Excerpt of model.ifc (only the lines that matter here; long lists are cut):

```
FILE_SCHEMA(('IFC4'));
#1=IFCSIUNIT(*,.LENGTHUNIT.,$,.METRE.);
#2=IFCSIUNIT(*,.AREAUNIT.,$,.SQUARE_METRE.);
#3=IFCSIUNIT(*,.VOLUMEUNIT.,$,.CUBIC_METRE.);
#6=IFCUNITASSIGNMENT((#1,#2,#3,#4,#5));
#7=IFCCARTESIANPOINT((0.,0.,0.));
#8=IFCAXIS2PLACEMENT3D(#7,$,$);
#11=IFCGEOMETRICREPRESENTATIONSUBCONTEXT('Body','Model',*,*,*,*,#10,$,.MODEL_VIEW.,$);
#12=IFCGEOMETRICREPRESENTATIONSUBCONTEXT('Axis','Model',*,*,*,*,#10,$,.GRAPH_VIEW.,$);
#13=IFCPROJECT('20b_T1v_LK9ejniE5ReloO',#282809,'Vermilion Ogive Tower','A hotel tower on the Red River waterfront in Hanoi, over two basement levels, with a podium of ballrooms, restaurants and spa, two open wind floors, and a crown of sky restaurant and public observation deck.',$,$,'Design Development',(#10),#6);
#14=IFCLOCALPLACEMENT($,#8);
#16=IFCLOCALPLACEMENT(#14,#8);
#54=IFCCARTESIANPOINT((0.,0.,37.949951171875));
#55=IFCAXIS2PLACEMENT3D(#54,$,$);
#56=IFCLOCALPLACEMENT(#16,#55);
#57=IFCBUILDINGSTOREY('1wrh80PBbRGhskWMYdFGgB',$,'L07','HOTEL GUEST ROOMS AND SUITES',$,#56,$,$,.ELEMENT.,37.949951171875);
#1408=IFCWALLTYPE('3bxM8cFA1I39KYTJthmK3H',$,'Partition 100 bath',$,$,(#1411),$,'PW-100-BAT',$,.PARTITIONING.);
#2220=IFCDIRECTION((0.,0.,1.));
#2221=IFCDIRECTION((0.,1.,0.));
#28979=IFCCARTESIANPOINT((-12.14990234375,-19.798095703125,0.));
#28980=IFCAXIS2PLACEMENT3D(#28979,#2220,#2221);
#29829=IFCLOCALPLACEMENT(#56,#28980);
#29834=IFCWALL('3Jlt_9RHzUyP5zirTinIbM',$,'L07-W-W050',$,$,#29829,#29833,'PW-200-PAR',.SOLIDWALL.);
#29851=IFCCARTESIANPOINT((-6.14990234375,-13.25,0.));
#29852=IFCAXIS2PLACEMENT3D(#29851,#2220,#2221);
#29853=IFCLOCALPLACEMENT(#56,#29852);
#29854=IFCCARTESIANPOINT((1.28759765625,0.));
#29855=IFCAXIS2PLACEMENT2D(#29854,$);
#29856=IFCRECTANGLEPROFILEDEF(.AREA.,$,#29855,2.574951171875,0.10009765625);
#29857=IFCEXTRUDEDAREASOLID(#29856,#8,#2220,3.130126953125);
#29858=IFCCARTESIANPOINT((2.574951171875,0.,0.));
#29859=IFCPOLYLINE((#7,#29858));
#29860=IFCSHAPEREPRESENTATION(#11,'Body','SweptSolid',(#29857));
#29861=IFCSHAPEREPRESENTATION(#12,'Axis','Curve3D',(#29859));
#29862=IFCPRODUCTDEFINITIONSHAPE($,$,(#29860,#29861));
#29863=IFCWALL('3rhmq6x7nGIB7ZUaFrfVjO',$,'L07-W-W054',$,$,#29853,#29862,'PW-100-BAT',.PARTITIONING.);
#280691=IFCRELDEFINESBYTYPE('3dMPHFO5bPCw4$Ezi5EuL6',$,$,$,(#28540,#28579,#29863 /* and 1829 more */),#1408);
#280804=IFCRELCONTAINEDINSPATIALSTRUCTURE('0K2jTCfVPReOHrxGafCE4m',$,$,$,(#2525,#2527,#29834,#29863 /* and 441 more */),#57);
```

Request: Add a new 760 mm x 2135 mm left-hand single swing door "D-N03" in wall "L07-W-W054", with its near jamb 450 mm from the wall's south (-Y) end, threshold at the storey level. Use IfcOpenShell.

```python
import numpy as np
import ifcopenshell
import ifcopenshell.api.feature
import ifcopenshell.api.geometry
import ifcopenshell.api.root
import ifcopenshell.api.spatial
import ifcopenshell.geom
import ifcopenshell.util.element
import ifcopenshell.util.placement
import ifcopenshell.util.representation
import ifcopenshell.util.shape
import ifcopenshell.util.unit

model = ifcopenshell.open("model.ifc")
unit_scale = ifcopenshell.util.unit.calculate_unit_scale(model)
settings = ifcopenshell.geom.settings()


def volume(element):
    """Net volume in cubic metres, openings subtracted."""
    shape = ifcopenshell.geom.create_shape(settings, element)
    return ifcopenshell.util.shape.get_volume(shape.geometry)


wall = model.by_id(29863)
storey = ifcopenshell.util.element.get_container(wall, ifc_class="IfcBuildingStorey")
context = ifcopenshell.util.representation.get_context(model, "Model", "Body", "MODEL_VIEW")
before = volume(wall)

width, height, from_end, sill = 0.76, 2.135, 0.45, 0.0  # metres

# The wall runs along its own X axis, and the end named is its -X end.
wall_shape = ifcopenshell.geom.create_shape(settings, wall)
x, y, z = ifcopenshell.util.shape.get_vertices(wall_shape.geometry).T
start = x.min() + from_end
face, thickness = float(y.min()), float(y.max() - y.min())
wall_matrix = ifcopenshell.util.placement.get_local_placement(wall.ObjectPlacement)
level = ifcopenshell.util.placement.get_local_placement(storey.ObjectPlacement)[2, 3]


def in_wall(x, y):
    """Placement at x, y metres in the wall's axes, at sill height."""
    matrix = wall_matrix.copy()
    matrix[:, 3] = wall_matrix @ np.array([x / unit_scale, y / unit_scale, 0.0, 1.0])
    matrix[2, 3] = level + sill / unit_scale
    return matrix


# Opening: a box that overshoots both wall faces by 50 mm.
opening = ifcopenshell.api.root.create_entity(model, ifc_class="IfcOpeningElement", predefined_type="OPENING")
box = ifcopenshell.api.geometry.add_wall_representation(
    model, context=context, length=width, height=height, thickness=thickness + 0.1
)
ifcopenshell.api.geometry.assign_representation(model, product=opening, representation=box)
ifcopenshell.api.geometry.edit_object_placement(model, product=opening, matrix=in_wall(start, face - 0.05), is_si=False)
ifcopenshell.api.feature.add_feature(model, feature=opening, element=wall)

door = ifcopenshell.api.root.create_entity(model, ifc_class="IfcDoor", name="D-N03", predefined_type="DOOR")
door.OverallWidth, door.OverallHeight = width / unit_scale, height / unit_scale
door.OperationType = "SINGLE_SWING_LEFT"
body = ifcopenshell.api.geometry.add_door_representation(
    model,
    context=context,
    overall_width=door.OverallWidth,
    overall_height=door.OverallHeight,
    operation_type="SINGLE_SWING_LEFT",
    lining_properties={"LiningDepth": thickness / unit_scale, "ThresholdDepth": thickness / unit_scale},
)
ifcopenshell.api.geometry.assign_representation(model, product=door, representation=body)
ifcopenshell.api.spatial.assign_container(model, products=[door], relating_structure=storey)
ifcopenshell.api.feature.add_filling(model, opening=opening, element=door)

# The lining spans the wall, so the door starts at the wall face.
ifcopenshell.api.geometry.edit_object_placement(model, product=door, matrix=in_wall(start, face), is_si=False)

after = volume(wall)

print(f"wall volume {before:.3f} -> {after:.3f} m3")

model.write("model_edited.ifc")
```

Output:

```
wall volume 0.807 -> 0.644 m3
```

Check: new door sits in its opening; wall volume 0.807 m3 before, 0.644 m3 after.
